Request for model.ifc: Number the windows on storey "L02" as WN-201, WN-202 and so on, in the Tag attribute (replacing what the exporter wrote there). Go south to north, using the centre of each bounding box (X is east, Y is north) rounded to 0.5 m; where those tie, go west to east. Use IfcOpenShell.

First a look at what the model holds.

```python
import ifcopenshell
import ifcopenshell.util.element
import ifcopenshell.util.placement

model = ifcopenshell.open("model.ifc")
print(model.schema)
storey = next(s for s in model.by_type("IfcBuildingStorey") if s.Name == "L02")
windows = [e for e in ifcopenshell.util.element.get_decomposition(storey) if e.is_a("IfcWindow")]
for e in sorted(windows, key=lambda e: e.id()):
    origin = ifcopenshell.util.placement.get_local_placement(e.ObjectPlacement)[:3, 3]
    print(e.id(), e.Tag, e.Name, origin.round(2) + 0.0, sep=" | ")
```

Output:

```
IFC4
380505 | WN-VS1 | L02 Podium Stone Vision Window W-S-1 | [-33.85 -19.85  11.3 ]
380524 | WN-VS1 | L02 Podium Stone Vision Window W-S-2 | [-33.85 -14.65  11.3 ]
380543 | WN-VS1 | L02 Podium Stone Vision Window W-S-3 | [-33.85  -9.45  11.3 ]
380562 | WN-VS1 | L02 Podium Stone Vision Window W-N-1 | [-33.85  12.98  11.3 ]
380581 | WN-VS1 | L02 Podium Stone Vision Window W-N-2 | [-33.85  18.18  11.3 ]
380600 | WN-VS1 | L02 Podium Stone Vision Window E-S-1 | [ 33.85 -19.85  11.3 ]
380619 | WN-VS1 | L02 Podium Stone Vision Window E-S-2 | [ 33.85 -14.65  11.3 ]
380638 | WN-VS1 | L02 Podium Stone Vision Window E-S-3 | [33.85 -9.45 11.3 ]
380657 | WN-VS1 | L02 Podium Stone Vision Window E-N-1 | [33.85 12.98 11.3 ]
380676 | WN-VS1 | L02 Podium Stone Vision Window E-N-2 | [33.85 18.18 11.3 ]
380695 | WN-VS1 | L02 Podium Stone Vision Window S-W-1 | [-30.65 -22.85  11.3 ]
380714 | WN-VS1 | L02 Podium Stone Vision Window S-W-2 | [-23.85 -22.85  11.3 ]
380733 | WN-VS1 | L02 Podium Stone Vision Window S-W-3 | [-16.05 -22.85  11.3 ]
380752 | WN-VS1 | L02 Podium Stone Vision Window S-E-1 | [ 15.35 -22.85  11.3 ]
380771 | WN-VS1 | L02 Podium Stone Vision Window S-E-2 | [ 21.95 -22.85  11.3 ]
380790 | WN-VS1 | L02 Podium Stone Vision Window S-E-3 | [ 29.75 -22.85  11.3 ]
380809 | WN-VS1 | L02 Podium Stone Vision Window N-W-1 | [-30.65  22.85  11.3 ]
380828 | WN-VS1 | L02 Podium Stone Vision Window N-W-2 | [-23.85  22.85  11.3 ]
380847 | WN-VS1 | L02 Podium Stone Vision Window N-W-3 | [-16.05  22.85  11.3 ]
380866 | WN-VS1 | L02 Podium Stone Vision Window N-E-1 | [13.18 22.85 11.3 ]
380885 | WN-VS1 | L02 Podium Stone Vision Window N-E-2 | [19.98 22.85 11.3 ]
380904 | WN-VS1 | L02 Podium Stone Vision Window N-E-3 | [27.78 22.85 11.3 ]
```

```python
import ifcopenshell
import ifcopenshell.geom
import ifcopenshell.util.element
import ifcopenshell.util.shape

model = ifcopenshell.open("model.ifc")
settings = ifcopenshell.geom.settings()
settings.set("use-world-coords", True)


def centre(element):
    shape = ifcopenshell.geom.create_shape(settings, element)
    return ifcopenshell.util.shape.get_bbox_centroid(shape.geometry)


storey = next(s for s in model.by_type("IfcBuildingStorey") if s.Name == "L02")
windows = [e for e in ifcopenshell.util.element.get_decomposition(storey) if e.is_a("IfcWindow")]

# Insertion points can sit at a corner or the storey origin, so sort by the geometry (in metres).
centres = {e: centre(e) for e in windows}
windows.sort(key=lambda e: (round(centres[e][1] / 0.5), centres[e][0]))

for i, e in enumerate(windows, start=1):
    number = f"WN-2{i:02d}"
    e.Tag = number
    print(e.id(), number)

model.write("model_v2.ifc")
```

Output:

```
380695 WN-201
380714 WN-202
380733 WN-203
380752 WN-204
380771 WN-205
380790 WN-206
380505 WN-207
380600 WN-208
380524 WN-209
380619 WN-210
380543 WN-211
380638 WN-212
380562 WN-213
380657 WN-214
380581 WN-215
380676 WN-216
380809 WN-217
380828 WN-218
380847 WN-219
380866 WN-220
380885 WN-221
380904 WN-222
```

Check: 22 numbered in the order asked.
